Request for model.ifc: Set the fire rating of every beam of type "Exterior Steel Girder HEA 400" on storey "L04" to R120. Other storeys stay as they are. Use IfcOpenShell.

First a look at what the model holds.

```python
import ifcopenshell
import ifcopenshell.util.element

model = ifcopenshell.open("model.ifc")
print(model.schema)
storey = next(s for s in model.by_type("IfcBuildingStorey") if s.Name == "L04")
beams = [e for e in ifcopenshell.util.element.get_decomposition(storey) if e.is_a("IfcBeam")]
seen = {}
for e in beams:
    element_type = ifcopenshell.util.element.get_type(e)
    key = (element_type.Name if element_type != e and element_type else None, ifcopenshell.util.element.get_pset(e, "Pset_BeamCommon", "FireRating"))
    seen[key] = seen.get(key, 0) + 1
for (name, value), count in sorted(seen.items(), key=str):
    print(count, "x", name, "|", value)
```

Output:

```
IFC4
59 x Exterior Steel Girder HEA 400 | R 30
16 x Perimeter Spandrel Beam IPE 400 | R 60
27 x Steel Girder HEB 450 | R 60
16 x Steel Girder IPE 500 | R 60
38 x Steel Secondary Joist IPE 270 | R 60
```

```python
import ifcopenshell
import ifcopenshell.api.pset
import ifcopenshell.util.element

model = ifcopenshell.open("model.ifc")

storey = next(s for s in model.by_type("IfcBuildingStorey") if s.Name == "L04")
beams = [e for e in ifcopenshell.util.element.get_decomposition(storey) if e.is_a("IfcBeam")]

count = 0
for e in beams:
    element_type = ifcopenshell.util.element.get_type(e)
    if element_type in (None, e) or element_type.Name != "Exterior Steel Girder HEA 400":
        continue
    # add_pset returns the element's existing set when there is one.
    pset = ifcopenshell.api.pset.add_pset(model, product=e, name="Pset_BeamCommon")
    ifcopenshell.api.pset.edit_pset(model, pset=pset, properties={"FireRating": "R120"})
    count += 1

print(count, "beams updated")

model.write("model-out.ifc")
```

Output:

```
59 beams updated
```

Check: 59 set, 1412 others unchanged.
